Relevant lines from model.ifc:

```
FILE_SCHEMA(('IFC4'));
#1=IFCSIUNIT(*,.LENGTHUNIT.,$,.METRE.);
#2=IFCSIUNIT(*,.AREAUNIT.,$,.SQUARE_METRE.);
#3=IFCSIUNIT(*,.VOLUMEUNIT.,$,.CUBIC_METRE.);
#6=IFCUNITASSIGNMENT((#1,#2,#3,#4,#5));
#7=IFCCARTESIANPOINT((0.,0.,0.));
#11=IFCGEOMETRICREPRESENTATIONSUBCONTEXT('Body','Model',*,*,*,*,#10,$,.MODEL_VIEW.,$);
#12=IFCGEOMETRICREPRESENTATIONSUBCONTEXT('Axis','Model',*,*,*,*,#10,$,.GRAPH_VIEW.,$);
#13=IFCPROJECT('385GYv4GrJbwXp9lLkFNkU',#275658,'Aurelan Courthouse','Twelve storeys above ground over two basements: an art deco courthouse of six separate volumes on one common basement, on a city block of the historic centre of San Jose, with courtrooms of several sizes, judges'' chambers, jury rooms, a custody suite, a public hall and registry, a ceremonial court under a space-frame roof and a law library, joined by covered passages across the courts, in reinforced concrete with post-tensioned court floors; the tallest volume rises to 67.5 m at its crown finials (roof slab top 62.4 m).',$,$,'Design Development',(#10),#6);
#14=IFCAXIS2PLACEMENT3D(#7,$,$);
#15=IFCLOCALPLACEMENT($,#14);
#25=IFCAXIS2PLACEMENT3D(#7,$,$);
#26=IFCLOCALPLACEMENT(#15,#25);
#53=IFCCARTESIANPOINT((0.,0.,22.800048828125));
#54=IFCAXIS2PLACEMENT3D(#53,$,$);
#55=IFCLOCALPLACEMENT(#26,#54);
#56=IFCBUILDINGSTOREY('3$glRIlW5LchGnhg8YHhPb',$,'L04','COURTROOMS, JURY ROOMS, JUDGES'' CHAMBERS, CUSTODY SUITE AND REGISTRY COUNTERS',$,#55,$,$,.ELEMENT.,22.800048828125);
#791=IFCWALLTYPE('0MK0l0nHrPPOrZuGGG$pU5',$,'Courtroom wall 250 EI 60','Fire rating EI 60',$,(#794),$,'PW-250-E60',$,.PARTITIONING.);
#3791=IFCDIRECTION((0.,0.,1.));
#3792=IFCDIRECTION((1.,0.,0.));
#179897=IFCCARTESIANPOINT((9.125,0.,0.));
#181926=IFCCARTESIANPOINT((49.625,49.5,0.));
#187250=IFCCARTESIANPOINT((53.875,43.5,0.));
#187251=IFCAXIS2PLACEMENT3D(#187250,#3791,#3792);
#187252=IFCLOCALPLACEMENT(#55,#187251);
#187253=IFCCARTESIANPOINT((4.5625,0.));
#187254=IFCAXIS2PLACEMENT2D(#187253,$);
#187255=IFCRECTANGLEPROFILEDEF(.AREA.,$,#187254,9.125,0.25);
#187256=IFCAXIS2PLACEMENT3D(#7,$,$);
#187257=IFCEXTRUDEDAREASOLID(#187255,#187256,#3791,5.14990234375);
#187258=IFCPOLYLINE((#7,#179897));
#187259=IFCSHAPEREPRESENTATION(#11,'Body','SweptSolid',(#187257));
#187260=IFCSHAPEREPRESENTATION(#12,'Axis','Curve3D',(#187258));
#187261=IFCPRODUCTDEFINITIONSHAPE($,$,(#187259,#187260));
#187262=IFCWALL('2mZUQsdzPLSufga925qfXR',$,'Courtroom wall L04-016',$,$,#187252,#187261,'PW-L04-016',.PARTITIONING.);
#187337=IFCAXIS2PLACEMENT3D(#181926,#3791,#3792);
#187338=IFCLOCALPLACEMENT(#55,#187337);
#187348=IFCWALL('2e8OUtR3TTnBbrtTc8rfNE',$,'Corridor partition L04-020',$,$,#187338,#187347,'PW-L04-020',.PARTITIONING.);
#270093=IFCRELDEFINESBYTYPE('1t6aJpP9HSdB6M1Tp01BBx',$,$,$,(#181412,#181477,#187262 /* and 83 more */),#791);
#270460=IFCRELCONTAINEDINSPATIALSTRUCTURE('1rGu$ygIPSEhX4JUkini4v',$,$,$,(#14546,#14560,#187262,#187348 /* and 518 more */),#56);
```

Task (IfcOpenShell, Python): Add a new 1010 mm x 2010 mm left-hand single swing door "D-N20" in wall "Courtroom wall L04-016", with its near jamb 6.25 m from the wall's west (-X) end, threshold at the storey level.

```python
import numpy as np
import ifcopenshell
import ifcopenshell.api.feature
import ifcopenshell.api.geometry
import ifcopenshell.api.root
import ifcopenshell.api.spatial
import ifcopenshell.geom
import ifcopenshell.util.element
import ifcopenshell.util.placement
import ifcopenshell.util.representation
import ifcopenshell.util.shape
import ifcopenshell.util.unit

model = ifcopenshell.open("model.ifc")
unit_scale = ifcopenshell.util.unit.calculate_unit_scale(model)
settings = ifcopenshell.geom.settings()


def volume(element):
    """Net volume in cubic metres, openings subtracted."""
    shape = ifcopenshell.geom.create_shape(settings, element)
    return ifcopenshell.util.shape.get_volume(shape.geometry)


wall = model.by_guid("2mZUQsdzPLSufga925qfXR")
storey = ifcopenshell.util.element.get_container(wall, ifc_class="IfcBuildingStorey")
context = ifcopenshell.util.representation.get_context(model, "Model", "Body", "MODEL_VIEW")
before = volume(wall)

width, height, from_end, sill = 1.01, 2.01, 6.25, 0.0  # metres

# The wall runs along its own X axis, and the end named is its -X end.
wall_shape = ifcopenshell.geom.create_shape(settings, wall)
x, y, z = ifcopenshell.util.shape.get_vertices(wall_shape.geometry).T
start = x.min() + from_end
face, thickness = float(y.min()), float(y.max() - y.min())
wall_matrix = ifcopenshell.util.placement.get_local_placement(wall.ObjectPlacement)
level = ifcopenshell.util.placement.get_local_placement(storey.ObjectPlacement)[2, 3]


def in_wall(x, y):
    """Placement at x, y metres in the wall's axes, at sill height."""
    matrix = wall_matrix.copy()
    matrix[:, 3] = wall_matrix @ np.array([x / unit_scale, y / unit_scale, 0.0, 1.0])
    matrix[2, 3] = level + sill / unit_scale
    return matrix


# Opening: a box that overshoots both wall faces by 50 mm.
opening = ifcopenshell.api.root.create_entity(model, ifc_class="IfcOpeningElement", predefined_type="OPENING")
box = ifcopenshell.api.geometry.add_wall_representation(
    model, context=context, length=width, height=height, thickness=thickness + 0.1
)
ifcopenshell.api.geometry.assign_representation(model, product=opening, representation=box)
ifcopenshell.api.geometry.edit_object_placement(model, product=opening, matrix=in_wall(start, face - 0.05), is_si=False)
ifcopenshell.api.feature.add_feature(model, feature=opening, element=wall)

door = ifcopenshell.api.root.create_entity(model, ifc_class="IfcDoor", name="D-N20", predefined_type="DOOR")
door.OverallWidth, door.OverallHeight = width / unit_scale, height / unit_scale
door.OperationType = "SINGLE_SWING_LEFT"
body = ifcopenshell.api.geometry.add_door_representation(
    model,
    context=context,
    overall_width=door.OverallWidth,
    overall_height=door.OverallHeight,
    operation_type="SINGLE_SWING_LEFT",
    lining_properties={"LiningDepth": thickness / unit_scale, "ThresholdDepth": thickness / unit_scale},
)
ifcopenshell.api.geometry.assign_representation(model, product=door, representation=body)
ifcopenshell.api.spatial.assign_container(model, products=[door], relating_structure=storey)
ifcopenshell.api.feature.add_filling(model, opening=opening, element=door)

# The lining spans the wall, so the door starts at the wall face.
ifcopenshell.api.geometry.edit_object_placement(model, product=door, matrix=in_wall(start, face), is_si=False)

after = volume(wall)

print(f"wall volume {before:.3f} -> {after:.3f} m3")

model.write("model-out.ifc")
```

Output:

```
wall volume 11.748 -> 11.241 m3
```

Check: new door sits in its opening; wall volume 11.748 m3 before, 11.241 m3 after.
